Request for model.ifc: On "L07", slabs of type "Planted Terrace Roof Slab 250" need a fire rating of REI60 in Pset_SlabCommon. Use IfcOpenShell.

First a look at what the model holds.

```python
import ifcopenshell
import ifcopenshell.util.element

model = ifcopenshell.open("model.ifc")
print(model.schema)
storey = next(s for s in model.by_type("IfcBuildingStorey") if s.Name == "L07")
slabs = [e for e in ifcopenshell.util.element.get_decomposition(storey) if e.is_a("IfcSlab")]
seen = {}
for e in slabs:
    element_type = ifcopenshell.util.element.get_type(e)
    key = (element_type.Name if element_type != e and element_type else None, ifcopenshell.util.element.get_pset(e, "Pset_SlabCommon", "FireRating"))
    seen[key] = seen.get(key, 0) + 1
for (name, value), count in sorted(seen.items(), key=str):
    print(count, "x", name, "|", value)
```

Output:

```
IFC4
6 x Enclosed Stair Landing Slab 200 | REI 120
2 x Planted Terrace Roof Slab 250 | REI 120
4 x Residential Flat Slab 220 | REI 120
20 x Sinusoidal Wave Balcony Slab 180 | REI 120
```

```python
import ifcopenshell
import ifcopenshell.api.pset
import ifcopenshell.util.element

model = ifcopenshell.open("model.ifc")

storey = next(s for s in model.by_type("IfcBuildingStorey") if s.Name == "L07")
slabs = [e for e in ifcopenshell.util.element.get_decomposition(storey) if e.is_a("IfcSlab")]

count = 0
for e in slabs:
    element_type = ifcopenshell.util.element.get_type(e)
    if element_type in (None, e) or element_type.Name != "Planted Terrace Roof Slab 250":
        continue
    # add_pset returns the element's existing set when there is one.
    pset = ifcopenshell.api.pset.add_pset(model, product=e, name="Pset_SlabCommon")
    ifcopenshell.api.pset.edit_pset(model, pset=pset, properties={"FireRating": "REI60"})
    count += 1

print(count, "slabs updated")

model.write("model_edited.ifc")
```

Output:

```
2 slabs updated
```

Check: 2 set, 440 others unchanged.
